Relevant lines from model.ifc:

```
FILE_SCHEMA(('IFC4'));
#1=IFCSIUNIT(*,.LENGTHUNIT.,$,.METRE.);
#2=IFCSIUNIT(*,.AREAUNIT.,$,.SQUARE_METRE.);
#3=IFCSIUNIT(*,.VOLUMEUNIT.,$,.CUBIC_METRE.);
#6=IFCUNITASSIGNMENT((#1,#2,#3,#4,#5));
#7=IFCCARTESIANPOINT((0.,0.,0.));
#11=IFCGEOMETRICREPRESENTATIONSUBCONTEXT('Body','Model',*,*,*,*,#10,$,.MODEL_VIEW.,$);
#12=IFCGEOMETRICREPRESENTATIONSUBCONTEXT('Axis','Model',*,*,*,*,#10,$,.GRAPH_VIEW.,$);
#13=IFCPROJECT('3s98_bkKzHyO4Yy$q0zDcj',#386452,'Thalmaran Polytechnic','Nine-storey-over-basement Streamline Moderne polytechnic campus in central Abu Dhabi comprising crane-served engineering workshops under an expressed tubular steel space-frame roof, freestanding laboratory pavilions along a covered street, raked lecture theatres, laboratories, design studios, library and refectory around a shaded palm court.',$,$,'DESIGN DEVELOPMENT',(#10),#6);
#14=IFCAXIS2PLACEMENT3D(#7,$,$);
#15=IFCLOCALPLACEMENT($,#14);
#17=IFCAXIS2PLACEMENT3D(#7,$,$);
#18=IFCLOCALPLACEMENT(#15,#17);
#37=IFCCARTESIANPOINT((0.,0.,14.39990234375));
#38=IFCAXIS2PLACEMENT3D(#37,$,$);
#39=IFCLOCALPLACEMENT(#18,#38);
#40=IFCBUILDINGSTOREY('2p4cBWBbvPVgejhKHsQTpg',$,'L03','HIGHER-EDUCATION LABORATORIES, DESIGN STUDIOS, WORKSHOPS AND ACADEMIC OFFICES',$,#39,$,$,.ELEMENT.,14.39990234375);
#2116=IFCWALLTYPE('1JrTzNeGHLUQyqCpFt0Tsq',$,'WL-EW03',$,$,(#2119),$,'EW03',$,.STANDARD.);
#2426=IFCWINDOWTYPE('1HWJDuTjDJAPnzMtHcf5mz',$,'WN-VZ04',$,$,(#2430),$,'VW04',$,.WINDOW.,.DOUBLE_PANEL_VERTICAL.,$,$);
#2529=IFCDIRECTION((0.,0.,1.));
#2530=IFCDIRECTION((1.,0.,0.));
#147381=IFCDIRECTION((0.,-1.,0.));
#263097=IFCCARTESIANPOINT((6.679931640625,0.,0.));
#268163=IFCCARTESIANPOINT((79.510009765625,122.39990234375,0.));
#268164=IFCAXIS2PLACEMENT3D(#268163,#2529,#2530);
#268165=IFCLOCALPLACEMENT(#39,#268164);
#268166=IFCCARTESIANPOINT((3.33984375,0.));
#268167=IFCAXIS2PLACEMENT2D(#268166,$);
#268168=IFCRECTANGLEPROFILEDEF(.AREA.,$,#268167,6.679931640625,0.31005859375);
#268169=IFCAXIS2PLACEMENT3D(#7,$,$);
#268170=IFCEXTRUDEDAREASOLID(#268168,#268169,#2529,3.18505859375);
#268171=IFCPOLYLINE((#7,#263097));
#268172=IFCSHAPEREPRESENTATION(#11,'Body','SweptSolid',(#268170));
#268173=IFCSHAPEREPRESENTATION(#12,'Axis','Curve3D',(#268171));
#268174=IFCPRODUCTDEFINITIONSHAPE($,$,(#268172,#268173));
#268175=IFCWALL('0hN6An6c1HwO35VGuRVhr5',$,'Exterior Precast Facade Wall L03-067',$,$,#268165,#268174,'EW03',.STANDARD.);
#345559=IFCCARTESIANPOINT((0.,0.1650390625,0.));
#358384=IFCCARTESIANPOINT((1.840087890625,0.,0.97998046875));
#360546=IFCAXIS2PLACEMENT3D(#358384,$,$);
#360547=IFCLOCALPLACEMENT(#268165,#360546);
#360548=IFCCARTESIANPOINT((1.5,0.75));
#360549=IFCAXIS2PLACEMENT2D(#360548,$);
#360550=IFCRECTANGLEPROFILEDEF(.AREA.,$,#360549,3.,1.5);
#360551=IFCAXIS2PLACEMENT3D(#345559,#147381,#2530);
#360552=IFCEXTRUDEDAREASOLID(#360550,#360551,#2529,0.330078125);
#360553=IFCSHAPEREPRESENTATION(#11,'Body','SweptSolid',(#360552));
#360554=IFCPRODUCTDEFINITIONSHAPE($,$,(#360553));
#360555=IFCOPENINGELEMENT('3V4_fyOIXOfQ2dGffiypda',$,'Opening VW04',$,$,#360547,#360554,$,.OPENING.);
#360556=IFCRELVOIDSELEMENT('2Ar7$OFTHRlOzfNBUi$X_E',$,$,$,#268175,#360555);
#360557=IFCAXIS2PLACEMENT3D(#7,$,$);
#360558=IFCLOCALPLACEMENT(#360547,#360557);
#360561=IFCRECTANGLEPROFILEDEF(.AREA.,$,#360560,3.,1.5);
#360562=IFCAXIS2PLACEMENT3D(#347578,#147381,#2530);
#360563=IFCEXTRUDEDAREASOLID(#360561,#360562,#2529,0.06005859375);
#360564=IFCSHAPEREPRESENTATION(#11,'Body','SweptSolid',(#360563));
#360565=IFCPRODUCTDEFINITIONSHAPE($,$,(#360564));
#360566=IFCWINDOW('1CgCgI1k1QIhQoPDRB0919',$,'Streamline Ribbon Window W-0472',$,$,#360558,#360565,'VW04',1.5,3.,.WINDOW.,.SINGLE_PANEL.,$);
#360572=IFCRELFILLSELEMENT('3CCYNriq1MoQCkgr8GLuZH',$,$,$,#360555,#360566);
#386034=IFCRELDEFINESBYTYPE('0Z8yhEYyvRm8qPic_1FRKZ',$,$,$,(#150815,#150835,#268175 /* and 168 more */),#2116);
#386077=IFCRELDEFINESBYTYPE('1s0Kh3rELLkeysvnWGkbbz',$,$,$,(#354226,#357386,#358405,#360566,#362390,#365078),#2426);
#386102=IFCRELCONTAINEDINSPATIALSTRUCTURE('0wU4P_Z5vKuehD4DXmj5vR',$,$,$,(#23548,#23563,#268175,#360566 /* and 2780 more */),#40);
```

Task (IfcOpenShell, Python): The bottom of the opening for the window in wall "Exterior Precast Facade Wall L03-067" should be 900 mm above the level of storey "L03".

```python
import numpy as np
import ifcopenshell
import ifcopenshell.api.geometry
import ifcopenshell.geom
import ifcopenshell.util.element
import ifcopenshell.util.placement
import ifcopenshell.util.shape
import ifcopenshell.util.unit

model = ifcopenshell.open("model.ifc")
unit_scale = ifcopenshell.util.unit.calculate_unit_scale(model)

window = model.by_id(360566)
opening = window.FillsVoids[0].RelatingOpeningElement
storey = ifcopenshell.util.element.get_container(window, ifc_class="IfcBuildingStorey")
level = ifcopenshell.util.placement.get_local_placement(storey.ObjectPlacement)[2, 3]

# The opening's origin need not be at the sill, so measure its lowest point.
shape = ifcopenshell.geom.create_shape(ifcopenshell.geom.settings(), opening)
bottom = ifcopenshell.util.shape.get_shape_bottom_elevation(shape, shape.geometry) / unit_scale
dz = level + 0.9 / unit_scale - bottom

shift = np.array([0.0, 0.0, dz])
# The window is placed relative to its opening, so it follows when the opening moves.
matrix = ifcopenshell.util.placement.get_local_placement(opening.ObjectPlacement)
matrix[:3, 3] += shift
ifcopenshell.api.geometry.edit_object_placement(
    model, product=opening, matrix=matrix, is_si=False, should_transform_children=True
)

print(f"moved by {dz * unit_scale:+.3f} m")

model.write("model-out.ifc")
```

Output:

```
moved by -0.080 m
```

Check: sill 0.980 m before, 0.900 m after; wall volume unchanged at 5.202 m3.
